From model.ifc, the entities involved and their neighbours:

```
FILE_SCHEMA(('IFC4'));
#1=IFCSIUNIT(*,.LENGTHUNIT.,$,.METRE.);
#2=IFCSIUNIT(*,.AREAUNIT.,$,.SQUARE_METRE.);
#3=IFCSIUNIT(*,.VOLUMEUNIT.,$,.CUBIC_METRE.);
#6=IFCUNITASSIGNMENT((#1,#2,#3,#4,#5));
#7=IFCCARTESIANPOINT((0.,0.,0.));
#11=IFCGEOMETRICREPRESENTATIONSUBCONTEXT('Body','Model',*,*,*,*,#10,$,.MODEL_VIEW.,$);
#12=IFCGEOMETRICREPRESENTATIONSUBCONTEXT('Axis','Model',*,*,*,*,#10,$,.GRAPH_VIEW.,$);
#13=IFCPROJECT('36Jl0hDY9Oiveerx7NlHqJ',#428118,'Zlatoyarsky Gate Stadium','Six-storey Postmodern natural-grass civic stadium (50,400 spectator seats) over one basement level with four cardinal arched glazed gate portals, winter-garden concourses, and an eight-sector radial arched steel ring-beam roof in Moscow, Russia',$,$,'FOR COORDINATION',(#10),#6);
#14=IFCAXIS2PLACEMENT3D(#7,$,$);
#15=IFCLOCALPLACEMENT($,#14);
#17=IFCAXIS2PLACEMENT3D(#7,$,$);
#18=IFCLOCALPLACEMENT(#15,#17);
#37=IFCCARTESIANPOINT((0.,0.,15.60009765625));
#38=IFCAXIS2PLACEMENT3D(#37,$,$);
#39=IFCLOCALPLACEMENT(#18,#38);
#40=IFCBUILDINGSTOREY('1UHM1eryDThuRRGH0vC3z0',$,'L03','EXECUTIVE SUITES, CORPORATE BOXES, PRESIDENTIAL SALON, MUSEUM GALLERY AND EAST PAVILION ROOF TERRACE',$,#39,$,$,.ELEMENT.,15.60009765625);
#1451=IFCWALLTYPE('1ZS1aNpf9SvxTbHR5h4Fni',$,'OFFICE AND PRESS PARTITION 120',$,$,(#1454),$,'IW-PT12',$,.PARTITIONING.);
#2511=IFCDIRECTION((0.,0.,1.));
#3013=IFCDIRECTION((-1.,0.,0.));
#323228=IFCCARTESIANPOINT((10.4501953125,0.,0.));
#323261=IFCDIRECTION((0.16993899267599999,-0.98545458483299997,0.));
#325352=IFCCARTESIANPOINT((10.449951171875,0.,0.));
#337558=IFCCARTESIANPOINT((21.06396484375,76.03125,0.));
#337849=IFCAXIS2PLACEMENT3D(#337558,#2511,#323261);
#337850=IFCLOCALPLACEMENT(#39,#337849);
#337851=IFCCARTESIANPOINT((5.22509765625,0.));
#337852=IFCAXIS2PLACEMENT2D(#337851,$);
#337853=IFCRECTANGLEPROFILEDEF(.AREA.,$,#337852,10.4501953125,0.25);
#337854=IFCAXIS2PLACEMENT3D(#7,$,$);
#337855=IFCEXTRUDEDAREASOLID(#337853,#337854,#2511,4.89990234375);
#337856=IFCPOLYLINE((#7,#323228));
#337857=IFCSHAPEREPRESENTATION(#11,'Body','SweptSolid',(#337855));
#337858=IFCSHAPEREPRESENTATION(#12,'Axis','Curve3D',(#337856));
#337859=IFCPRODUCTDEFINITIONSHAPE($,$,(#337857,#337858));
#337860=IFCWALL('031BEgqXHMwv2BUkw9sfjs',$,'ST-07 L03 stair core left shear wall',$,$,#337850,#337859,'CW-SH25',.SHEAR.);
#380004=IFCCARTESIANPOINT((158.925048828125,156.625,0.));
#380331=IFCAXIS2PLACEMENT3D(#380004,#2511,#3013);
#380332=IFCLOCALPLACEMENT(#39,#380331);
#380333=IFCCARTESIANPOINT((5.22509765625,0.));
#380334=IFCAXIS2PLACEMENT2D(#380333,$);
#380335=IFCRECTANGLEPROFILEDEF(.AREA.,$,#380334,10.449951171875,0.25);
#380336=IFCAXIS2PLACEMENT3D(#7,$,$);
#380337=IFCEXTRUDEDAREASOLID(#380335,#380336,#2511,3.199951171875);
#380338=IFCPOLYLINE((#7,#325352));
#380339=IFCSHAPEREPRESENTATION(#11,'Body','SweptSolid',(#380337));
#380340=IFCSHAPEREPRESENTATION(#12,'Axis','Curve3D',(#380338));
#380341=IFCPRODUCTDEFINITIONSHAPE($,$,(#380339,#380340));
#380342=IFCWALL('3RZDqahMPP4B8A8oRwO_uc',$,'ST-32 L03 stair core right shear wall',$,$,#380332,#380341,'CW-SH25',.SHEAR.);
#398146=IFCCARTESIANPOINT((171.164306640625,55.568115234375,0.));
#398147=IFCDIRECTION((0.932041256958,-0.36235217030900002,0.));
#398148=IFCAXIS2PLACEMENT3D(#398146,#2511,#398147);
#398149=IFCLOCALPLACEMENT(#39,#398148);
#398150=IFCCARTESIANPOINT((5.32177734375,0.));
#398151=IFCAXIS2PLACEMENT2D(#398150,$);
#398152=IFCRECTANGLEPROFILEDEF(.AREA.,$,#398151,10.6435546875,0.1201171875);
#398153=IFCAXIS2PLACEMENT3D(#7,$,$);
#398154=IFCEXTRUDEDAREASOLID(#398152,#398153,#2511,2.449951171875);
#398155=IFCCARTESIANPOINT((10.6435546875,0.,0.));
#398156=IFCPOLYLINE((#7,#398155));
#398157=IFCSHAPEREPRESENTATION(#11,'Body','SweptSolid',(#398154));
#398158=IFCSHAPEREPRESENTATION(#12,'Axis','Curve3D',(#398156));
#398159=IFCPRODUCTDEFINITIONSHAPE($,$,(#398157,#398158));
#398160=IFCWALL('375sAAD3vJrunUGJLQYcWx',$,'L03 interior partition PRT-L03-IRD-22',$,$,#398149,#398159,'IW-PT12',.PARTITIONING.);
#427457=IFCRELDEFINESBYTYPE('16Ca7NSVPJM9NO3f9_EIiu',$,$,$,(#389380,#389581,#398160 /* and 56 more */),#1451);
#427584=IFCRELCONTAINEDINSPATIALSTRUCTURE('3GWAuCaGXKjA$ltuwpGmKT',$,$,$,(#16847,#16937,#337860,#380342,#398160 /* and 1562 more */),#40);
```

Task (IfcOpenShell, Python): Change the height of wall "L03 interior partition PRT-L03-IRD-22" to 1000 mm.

```python
import ifcopenshell
import ifcopenshell.geom
import ifcopenshell.util.representation
import ifcopenshell.util.shape

model = ifcopenshell.open("model.ifc")
settings = ifcopenshell.geom.settings()


def volume(element):
    """Net volume in cubic metres, openings subtracted."""
    shape = ifcopenshell.geom.create_shape(settings, element)
    return ifcopenshell.util.shape.get_volume(shape.geometry)


wall = model.by_id(398160)
before = volume(wall)

body = ifcopenshell.util.representation.get_representation(wall, "Model", "Body")
solid = body.Items[0]
old_height = solid.Depth
solid.Depth = 1.0
after = volume(wall)

print(f"height {old_height:g} -> {solid.Depth:g}, volume {before:.3f} -> {after:.3f} m3")

model.write("model_updated.ifc")
```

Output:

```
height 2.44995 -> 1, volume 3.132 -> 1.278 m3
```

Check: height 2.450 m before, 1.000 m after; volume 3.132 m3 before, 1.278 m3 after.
